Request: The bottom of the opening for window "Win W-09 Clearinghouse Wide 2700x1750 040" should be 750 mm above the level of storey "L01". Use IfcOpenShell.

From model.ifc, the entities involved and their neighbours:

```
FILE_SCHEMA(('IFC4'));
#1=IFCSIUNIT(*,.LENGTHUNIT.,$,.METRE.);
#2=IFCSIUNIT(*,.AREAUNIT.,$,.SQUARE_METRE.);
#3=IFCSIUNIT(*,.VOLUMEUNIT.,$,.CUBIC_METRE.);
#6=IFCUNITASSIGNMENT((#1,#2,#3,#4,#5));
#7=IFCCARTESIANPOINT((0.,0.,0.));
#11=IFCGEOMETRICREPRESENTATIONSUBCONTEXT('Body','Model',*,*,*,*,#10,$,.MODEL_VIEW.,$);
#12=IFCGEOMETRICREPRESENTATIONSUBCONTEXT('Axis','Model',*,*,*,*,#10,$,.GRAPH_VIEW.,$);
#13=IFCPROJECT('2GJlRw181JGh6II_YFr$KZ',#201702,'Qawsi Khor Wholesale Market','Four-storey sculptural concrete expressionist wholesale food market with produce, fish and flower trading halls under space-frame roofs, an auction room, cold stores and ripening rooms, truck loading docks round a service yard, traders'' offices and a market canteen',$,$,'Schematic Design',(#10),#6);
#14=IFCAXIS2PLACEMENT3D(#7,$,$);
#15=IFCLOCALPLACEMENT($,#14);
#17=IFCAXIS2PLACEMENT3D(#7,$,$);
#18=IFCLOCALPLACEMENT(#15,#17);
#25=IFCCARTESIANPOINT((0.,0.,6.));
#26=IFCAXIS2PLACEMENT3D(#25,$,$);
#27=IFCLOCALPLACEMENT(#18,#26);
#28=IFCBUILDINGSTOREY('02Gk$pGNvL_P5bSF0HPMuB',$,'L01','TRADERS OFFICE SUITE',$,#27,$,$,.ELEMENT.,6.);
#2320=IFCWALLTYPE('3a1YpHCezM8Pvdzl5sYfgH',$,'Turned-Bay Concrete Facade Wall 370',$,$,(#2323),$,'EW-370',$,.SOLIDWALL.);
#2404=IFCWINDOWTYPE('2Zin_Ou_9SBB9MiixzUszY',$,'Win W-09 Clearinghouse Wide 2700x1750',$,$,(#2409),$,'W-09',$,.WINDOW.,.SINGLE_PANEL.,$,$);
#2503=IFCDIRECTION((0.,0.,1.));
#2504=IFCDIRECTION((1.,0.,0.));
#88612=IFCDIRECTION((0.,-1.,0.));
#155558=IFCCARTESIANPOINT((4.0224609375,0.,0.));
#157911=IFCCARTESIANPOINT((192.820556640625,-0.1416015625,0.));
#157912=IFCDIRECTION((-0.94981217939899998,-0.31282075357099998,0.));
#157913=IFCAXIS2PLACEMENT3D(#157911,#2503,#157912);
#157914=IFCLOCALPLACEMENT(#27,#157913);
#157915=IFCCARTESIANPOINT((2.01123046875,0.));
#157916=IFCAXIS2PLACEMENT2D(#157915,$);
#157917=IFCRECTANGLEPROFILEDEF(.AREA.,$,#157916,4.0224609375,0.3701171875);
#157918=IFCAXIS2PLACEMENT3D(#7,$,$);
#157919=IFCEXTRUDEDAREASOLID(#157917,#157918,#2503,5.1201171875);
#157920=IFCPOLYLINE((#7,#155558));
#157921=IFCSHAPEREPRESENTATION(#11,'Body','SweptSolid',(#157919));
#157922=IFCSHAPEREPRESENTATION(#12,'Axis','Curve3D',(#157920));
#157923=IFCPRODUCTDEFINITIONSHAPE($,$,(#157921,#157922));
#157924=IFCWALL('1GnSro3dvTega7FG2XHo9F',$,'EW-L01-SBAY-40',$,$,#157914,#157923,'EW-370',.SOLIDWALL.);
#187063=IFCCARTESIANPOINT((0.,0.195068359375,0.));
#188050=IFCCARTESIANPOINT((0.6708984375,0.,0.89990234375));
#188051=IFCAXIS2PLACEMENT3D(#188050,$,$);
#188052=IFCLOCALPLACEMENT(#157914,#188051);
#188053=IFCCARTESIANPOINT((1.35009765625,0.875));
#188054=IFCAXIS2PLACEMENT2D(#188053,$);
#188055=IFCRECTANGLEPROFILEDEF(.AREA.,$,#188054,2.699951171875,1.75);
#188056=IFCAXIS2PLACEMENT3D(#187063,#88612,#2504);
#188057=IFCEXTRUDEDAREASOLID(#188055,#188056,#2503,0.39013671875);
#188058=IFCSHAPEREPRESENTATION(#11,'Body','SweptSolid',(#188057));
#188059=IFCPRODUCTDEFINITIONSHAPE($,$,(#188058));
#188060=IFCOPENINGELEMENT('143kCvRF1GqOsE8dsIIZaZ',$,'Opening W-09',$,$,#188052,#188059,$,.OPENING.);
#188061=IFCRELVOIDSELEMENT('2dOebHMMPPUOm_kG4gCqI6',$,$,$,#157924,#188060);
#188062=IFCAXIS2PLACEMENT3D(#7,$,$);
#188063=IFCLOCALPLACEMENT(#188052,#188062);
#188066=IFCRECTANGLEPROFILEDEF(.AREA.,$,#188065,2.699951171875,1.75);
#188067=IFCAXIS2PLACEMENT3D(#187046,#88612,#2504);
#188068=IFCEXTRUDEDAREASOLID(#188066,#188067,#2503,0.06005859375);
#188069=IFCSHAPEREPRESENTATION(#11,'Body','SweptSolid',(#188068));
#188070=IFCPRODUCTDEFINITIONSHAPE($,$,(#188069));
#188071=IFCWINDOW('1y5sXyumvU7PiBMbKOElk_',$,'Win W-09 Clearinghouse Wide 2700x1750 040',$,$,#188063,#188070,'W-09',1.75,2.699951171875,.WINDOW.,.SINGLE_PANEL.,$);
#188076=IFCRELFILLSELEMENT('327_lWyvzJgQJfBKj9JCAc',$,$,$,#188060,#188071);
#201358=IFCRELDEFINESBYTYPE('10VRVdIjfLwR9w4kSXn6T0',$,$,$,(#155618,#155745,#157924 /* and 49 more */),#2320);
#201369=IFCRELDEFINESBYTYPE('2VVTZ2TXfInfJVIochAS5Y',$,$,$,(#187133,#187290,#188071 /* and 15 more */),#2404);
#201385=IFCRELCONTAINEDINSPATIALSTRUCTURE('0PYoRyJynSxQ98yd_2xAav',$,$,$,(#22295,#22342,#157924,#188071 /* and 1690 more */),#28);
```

```python
import numpy as np
import ifcopenshell
import ifcopenshell.api.geometry
import ifcopenshell.geom
import ifcopenshell.util.element
import ifcopenshell.util.placement
import ifcopenshell.util.shape
import ifcopenshell.util.unit

model = ifcopenshell.open("model.ifc")
unit_scale = ifcopenshell.util.unit.calculate_unit_scale(model)

window = model.by_guid("1y5sXyumvU7PiBMbKOElk_")
opening = window.FillsVoids[0].RelatingOpeningElement
storey = ifcopenshell.util.element.get_container(window, ifc_class="IfcBuildingStorey")
level = ifcopenshell.util.placement.get_local_placement(storey.ObjectPlacement)[2, 3]

# The opening's origin need not be at the sill, so measure its lowest point.
shape = ifcopenshell.geom.create_shape(ifcopenshell.geom.settings(), opening)
bottom = ifcopenshell.util.shape.get_shape_bottom_elevation(shape, shape.geometry) / unit_scale
dz = level + 0.75 - bottom

shift = np.array([0.0, 0.0, dz])
# The window is placed relative to its opening, so it follows when the opening moves.
matrix = ifcopenshell.util.placement.get_local_placement(opening.ObjectPlacement)
matrix[:3, 3] += shift
ifcopenshell.api.geometry.edit_object_placement(
    model, product=opening, matrix=matrix, is_si=False, should_transform_children=True
)

print(f"moved by {dz * unit_scale:+.3f} m")

model.write("model_v2.ifc")
```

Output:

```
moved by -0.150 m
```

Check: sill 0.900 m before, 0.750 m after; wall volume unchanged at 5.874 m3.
